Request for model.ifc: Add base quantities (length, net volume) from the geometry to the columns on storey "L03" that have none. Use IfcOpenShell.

First a look at what the model holds.

```python
import ifcopenshell
import ifcopenshell.util.element
import ifcopenshell.util.unit

model = ifcopenshell.open("model.ifc")
print(model.schema)
for unit_type in ("LENGTHUNIT", "AREAUNIT", "VOLUMEUNIT"):
    print(unit_type, ifcopenshell.util.unit.calculate_unit_scale(model, unit_type))
storey = next(s for s in model.by_type("IfcBuildingStorey") if s.Name == "L03")
columns = [e for e in ifcopenshell.util.element.get_decomposition(storey) if e.is_a("IfcColumn")]
for e in sorted(columns, key=lambda e: e.id()):
    print(e.id(), e.is_a(), e.Name, list(ifcopenshell.util.element.get_psets(e, qtos_only=True)), sep=" | ")
```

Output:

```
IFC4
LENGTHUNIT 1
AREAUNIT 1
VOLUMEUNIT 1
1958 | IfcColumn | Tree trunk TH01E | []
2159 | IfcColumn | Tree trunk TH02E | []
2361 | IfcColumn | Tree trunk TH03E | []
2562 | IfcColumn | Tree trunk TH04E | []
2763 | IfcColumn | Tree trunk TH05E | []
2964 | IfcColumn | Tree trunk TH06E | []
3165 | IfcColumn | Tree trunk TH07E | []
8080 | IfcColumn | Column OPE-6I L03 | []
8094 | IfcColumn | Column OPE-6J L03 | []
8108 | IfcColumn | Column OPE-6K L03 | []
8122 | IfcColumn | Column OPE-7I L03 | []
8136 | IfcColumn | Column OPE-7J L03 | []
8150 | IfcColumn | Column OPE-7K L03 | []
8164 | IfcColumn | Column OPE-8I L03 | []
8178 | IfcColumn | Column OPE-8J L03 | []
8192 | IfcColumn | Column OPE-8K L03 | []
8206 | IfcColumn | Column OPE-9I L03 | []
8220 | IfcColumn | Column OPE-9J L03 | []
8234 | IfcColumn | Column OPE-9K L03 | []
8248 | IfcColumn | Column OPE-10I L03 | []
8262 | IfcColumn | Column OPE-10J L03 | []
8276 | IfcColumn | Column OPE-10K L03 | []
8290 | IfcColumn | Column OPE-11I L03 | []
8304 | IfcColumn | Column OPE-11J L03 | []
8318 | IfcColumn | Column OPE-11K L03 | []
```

```python
import ifcopenshell
import ifcopenshell.api.pset
import ifcopenshell.geom
import ifcopenshell.util.element
import ifcopenshell.util.shape
import ifcopenshell.util.unit

model = ifcopenshell.open("model.ifc")
unit_scale = ifcopenshell.util.unit.calculate_unit_scale(model)
volume_scale = ifcopenshell.util.unit.calculate_unit_scale(model, "VOLUMEUNIT")
settings = ifcopenshell.geom.settings()

storey = next(s for s in model.by_type("IfcBuildingStorey") if s.Name == "L03")
columns = [e for e in ifcopenshell.util.element.get_decomposition(storey) if e.is_a("IfcColumn")]

for e in sorted(columns, key=lambda e: e.id()):
    if ifcopenshell.util.element.get_psets(e, qtos_only=True, should_inherit=False):
        continue
    # Geometry comes back in metres, in the element's own axes.
    shape = ifcopenshell.geom.create_shape(settings, e)
    values = {
        "Length": ifcopenshell.util.shape.get_z(shape.geometry) / unit_scale,
        "NetVolume": ifcopenshell.util.shape.get_volume(shape.geometry) / volume_scale,
    }
    qto = ifcopenshell.api.pset.add_qto(model, product=e, name="Qto_ColumnBaseQuantities")
    ifcopenshell.api.pset.edit_qto(model, qto=qto, properties=values)
    print(e.id(), {k: round(v, 3) for k, v in values.items()})

model.write("model-out.ifc")
```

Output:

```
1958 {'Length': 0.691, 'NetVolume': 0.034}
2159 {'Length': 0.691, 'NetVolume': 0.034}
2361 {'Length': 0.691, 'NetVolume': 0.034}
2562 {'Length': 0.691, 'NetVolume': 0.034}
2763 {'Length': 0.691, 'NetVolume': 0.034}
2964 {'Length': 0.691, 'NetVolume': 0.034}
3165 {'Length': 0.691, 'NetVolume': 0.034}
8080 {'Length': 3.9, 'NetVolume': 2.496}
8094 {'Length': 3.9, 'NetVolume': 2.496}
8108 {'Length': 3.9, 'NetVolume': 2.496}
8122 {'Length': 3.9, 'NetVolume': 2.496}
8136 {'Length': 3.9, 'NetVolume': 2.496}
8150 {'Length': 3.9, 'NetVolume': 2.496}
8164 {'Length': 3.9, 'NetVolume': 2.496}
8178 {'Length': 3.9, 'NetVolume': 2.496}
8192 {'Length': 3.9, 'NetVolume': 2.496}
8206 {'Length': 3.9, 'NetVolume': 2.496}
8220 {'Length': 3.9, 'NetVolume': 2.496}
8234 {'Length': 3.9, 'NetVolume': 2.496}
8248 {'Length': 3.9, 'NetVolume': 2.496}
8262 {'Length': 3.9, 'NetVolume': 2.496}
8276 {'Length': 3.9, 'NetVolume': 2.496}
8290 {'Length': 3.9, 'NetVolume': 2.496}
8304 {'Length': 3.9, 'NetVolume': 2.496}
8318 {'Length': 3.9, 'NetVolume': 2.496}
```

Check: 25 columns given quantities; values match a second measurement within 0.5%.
